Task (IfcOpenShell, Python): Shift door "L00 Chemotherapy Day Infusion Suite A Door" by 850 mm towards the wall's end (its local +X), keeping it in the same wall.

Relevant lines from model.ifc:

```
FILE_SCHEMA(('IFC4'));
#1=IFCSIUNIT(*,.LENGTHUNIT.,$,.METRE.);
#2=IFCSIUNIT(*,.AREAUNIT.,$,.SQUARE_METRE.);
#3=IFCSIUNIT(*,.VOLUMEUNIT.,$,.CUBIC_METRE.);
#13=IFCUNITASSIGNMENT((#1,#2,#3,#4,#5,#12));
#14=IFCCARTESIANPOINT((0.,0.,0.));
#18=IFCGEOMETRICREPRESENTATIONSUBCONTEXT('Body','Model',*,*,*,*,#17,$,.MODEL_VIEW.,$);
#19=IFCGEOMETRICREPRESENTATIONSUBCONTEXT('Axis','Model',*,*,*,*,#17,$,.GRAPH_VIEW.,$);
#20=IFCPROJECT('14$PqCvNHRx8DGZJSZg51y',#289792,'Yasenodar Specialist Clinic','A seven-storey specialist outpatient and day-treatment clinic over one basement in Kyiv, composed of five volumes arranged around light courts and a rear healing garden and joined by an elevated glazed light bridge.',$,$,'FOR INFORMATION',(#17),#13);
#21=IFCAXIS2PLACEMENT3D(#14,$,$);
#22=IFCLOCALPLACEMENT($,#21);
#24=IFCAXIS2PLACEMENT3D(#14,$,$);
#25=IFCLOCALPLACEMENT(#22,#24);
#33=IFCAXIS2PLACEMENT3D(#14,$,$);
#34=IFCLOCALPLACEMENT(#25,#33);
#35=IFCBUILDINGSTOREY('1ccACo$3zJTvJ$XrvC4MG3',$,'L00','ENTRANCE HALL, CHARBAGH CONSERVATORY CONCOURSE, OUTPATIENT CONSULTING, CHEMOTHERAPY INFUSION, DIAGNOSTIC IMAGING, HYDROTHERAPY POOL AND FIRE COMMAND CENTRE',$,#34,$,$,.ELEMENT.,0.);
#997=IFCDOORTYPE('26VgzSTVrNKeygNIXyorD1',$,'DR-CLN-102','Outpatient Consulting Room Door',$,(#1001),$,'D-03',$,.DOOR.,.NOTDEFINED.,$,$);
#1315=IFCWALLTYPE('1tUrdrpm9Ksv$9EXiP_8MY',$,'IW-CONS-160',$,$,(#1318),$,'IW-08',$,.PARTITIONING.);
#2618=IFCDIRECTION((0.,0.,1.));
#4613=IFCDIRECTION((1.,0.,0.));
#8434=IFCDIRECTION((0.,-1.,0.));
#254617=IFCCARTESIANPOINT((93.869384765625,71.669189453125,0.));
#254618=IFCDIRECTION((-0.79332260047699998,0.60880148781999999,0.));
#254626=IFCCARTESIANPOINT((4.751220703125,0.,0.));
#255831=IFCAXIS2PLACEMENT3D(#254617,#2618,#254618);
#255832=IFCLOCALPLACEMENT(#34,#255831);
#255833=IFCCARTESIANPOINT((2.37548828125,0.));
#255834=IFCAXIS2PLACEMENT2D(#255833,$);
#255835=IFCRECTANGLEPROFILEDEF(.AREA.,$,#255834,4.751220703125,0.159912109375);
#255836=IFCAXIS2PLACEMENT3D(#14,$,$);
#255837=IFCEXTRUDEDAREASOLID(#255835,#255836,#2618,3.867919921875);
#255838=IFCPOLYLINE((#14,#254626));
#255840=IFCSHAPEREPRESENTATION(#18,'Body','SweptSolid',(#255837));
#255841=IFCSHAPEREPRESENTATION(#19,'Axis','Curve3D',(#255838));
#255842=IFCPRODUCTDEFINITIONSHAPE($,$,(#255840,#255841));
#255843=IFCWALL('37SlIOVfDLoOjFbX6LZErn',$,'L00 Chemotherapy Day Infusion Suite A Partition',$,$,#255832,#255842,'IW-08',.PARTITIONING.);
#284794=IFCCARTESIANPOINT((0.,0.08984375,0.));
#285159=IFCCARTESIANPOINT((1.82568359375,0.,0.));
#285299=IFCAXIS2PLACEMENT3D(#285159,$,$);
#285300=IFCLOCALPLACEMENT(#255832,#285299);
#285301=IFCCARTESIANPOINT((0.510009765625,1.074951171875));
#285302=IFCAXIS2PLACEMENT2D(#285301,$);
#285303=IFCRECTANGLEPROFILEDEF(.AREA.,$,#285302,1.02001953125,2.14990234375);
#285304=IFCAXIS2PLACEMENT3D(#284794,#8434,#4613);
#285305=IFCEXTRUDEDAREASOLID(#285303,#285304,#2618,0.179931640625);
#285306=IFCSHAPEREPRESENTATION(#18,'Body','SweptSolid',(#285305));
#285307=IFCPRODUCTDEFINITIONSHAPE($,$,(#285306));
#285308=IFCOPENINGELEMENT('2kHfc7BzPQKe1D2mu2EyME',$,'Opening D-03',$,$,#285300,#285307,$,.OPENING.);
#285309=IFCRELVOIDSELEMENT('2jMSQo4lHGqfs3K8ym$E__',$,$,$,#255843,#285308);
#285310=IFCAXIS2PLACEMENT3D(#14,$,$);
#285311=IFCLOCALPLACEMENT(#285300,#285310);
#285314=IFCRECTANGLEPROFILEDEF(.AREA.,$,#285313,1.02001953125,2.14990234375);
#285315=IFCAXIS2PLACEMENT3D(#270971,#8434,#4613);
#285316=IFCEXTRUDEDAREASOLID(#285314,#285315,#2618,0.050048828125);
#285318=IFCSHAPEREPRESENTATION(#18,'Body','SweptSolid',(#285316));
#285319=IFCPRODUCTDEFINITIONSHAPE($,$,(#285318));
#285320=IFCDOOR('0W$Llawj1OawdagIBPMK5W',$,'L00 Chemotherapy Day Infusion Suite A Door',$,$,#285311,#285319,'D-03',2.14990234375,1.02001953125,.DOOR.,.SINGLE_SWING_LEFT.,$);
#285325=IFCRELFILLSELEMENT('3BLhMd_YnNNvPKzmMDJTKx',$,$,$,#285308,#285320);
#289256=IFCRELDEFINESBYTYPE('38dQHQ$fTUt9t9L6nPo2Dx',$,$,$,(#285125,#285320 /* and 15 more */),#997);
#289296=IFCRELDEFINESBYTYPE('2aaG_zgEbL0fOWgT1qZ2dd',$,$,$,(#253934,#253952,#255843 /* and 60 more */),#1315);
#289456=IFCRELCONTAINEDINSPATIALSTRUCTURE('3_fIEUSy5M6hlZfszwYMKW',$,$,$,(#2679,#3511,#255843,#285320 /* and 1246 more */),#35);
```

```python
import ifcopenshell
import ifcopenshell.api.geometry
import ifcopenshell.util.placement
import ifcopenshell.util.unit

model = ifcopenshell.open("model.ifc")
unit_scale = ifcopenshell.util.unit.calculate_unit_scale(model)

door = model.by_guid("0W$Llawj1OawdagIBPMK5W")
opening = door.FillsVoids[0].RelatingOpeningElement
wall = opening.VoidsElements[0].RelatingBuildingElement

wall_matrix = ifcopenshell.util.placement.get_local_placement(wall.ObjectPlacement)
shift = wall_matrix[:3, 0] * 0.85 / unit_scale
before = ifcopenshell.util.placement.get_local_placement(door.ObjectPlacement)[:3, 3].copy()

# The door is placed relative to its opening, so it follows when the opening moves.
matrix = ifcopenshell.util.placement.get_local_placement(opening.ObjectPlacement)
matrix[:3, 3] += shift
ifcopenshell.api.geometry.edit_object_placement(
    model, product=opening, matrix=matrix, is_si=False, should_transform_children=True
)

after = ifcopenshell.util.placement.get_local_placement(door.ObjectPlacement)[:3, 3]
print("door moved by", (after - before).round(3) + 0.0)

model.write("model_updated.ifc")
```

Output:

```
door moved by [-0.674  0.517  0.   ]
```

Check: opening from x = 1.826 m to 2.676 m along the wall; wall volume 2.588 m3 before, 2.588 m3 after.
